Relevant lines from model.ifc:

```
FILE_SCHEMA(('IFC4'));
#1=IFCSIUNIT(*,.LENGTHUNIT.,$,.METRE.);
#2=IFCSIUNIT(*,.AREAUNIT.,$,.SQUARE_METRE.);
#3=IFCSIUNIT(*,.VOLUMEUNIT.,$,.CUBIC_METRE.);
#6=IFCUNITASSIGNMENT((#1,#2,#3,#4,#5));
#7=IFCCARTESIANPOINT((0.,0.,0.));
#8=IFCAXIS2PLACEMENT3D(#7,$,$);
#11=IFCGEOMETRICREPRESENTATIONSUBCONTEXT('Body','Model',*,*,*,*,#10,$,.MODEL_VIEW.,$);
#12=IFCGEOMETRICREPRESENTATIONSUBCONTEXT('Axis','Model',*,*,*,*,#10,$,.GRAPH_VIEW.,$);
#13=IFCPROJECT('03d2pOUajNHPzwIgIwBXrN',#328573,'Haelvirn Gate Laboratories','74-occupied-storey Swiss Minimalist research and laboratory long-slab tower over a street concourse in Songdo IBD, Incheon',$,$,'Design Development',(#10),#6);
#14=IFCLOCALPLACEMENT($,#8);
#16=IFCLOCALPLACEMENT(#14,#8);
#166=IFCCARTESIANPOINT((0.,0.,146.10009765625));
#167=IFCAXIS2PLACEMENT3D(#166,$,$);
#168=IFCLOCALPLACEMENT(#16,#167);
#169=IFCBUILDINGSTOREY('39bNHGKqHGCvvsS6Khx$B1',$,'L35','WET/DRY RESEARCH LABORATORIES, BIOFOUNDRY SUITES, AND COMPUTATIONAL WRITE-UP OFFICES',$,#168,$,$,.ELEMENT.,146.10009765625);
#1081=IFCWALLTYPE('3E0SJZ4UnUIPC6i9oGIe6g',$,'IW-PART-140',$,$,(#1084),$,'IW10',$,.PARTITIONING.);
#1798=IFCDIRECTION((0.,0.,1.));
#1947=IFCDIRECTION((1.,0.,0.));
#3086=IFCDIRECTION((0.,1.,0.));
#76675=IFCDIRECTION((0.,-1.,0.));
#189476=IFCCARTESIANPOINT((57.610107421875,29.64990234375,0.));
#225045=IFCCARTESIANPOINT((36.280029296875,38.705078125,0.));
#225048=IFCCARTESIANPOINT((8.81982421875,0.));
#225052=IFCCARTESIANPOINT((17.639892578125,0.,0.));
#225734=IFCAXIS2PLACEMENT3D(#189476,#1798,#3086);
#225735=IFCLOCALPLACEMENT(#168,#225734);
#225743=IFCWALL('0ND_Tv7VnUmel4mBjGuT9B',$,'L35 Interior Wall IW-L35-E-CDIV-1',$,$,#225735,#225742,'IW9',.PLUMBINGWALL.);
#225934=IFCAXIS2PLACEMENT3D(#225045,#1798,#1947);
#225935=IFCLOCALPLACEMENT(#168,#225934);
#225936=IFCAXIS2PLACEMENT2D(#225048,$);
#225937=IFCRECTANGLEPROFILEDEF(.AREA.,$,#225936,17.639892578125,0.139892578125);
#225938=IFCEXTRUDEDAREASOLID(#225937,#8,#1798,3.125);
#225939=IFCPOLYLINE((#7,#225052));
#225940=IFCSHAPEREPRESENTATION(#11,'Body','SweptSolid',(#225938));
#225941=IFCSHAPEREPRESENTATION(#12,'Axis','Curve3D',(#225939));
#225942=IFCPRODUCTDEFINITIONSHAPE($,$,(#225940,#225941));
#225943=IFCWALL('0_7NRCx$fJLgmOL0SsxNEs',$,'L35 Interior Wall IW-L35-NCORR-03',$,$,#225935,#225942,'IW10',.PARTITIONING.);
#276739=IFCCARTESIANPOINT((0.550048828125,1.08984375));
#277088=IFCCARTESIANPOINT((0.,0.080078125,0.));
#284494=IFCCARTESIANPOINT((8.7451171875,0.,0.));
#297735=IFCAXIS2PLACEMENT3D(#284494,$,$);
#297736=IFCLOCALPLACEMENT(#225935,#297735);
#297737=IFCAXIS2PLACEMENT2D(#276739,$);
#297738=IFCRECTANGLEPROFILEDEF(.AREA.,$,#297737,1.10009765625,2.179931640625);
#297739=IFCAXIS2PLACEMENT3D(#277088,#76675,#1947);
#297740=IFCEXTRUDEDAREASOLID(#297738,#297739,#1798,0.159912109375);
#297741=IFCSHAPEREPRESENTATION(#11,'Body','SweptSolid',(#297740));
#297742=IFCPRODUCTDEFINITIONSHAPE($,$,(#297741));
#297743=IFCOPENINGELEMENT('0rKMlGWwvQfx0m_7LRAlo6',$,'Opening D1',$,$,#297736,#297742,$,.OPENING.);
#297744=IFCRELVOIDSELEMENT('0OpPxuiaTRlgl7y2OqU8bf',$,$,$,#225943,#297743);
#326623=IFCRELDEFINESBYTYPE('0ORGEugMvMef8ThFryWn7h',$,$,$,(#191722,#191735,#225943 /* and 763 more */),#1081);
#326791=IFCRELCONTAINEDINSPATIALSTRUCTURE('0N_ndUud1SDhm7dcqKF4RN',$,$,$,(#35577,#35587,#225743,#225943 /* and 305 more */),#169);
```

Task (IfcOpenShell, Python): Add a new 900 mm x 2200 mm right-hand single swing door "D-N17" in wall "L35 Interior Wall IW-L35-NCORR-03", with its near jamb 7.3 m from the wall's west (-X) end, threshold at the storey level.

```python
import numpy as np
import ifcopenshell
import ifcopenshell.api.feature
import ifcopenshell.api.geometry
import ifcopenshell.api.root
import ifcopenshell.api.spatial
import ifcopenshell.geom
import ifcopenshell.util.element
import ifcopenshell.util.placement
import ifcopenshell.util.representation
import ifcopenshell.util.shape
import ifcopenshell.util.unit

model = ifcopenshell.open("model.ifc")
unit_scale = ifcopenshell.util.unit.calculate_unit_scale(model)
settings = ifcopenshell.geom.settings()


def volume(element):
    """Net volume in cubic metres, openings subtracted."""
    shape = ifcopenshell.geom.create_shape(settings, element)
    return ifcopenshell.util.shape.get_volume(shape.geometry)


wall = model.by_guid("0_7NRCx$fJLgmOL0SsxNEs")
storey = ifcopenshell.util.element.get_container(wall, ifc_class="IfcBuildingStorey")
context = ifcopenshell.util.representation.get_context(model, "Model", "Body", "MODEL_VIEW")
before = volume(wall)

width, height, from_end, sill = 0.9, 2.2, 7.3, 0.0  # metres

# The wall runs along its own X axis, and the end named is its -X end.
wall_shape = ifcopenshell.geom.create_shape(settings, wall)
x, y, z = ifcopenshell.util.shape.get_vertices(wall_shape.geometry).T
start = x.min() + from_end
face, thickness = float(y.min()), float(y.max() - y.min())
wall_matrix = ifcopenshell.util.placement.get_local_placement(wall.ObjectPlacement)
level = ifcopenshell.util.placement.get_local_placement(storey.ObjectPlacement)[2, 3]


def in_wall(x, y):
    """Placement at x, y metres in the wall's axes, at sill height."""
    matrix = wall_matrix.copy()
    matrix[:, 3] = wall_matrix @ np.array([x / unit_scale, y / unit_scale, 0.0, 1.0])
    matrix[2, 3] = level + sill / unit_scale
    return matrix


# Opening: a box that overshoots both wall faces by 50 mm.
opening = ifcopenshell.api.root.create_entity(model, ifc_class="IfcOpeningElement", predefined_type="OPENING")
box = ifcopenshell.api.geometry.add_wall_representation(
    model, context=context, length=width, height=height, thickness=thickness + 0.1
)
ifcopenshell.api.geometry.assign_representation(model, product=opening, representation=box)
ifcopenshell.api.geometry.edit_object_placement(model, product=opening, matrix=in_wall(start, face - 0.05), is_si=False)
ifcopenshell.api.feature.add_feature(model, feature=opening, element=wall)

door = ifcopenshell.api.root.create_entity(model, ifc_class="IfcDoor", name="D-N17", predefined_type="DOOR")
door.OverallWidth, door.OverallHeight = width / unit_scale, height / unit_scale
door.OperationType = "SINGLE_SWING_RIGHT"
body = ifcopenshell.api.geometry.add_door_representation(
    model,
    context=context,
    overall_width=door.OverallWidth,
    overall_height=door.OverallHeight,
    operation_type="SINGLE_SWING_RIGHT",
    lining_properties={"LiningDepth": thickness / unit_scale, "ThresholdDepth": thickness / unit_scale},
)
ifcopenshell.api.geometry.assign_representation(model, product=door, representation=body)
ifcopenshell.api.spatial.assign_container(model, products=[door], relating_structure=storey)
ifcopenshell.api.feature.add_filling(model, opening=opening, element=door)

# The lining spans the wall, so the door starts at the wall face.
ifcopenshell.api.geometry.edit_object_placement(model, product=door, matrix=in_wall(start, face), is_si=False)

after = volume(wall)

print(f"wall volume {before:.3f} -> {after:.3f} m3")

model.write("model_updated.ifc")
```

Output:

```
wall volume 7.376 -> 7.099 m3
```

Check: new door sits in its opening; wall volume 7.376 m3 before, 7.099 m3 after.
